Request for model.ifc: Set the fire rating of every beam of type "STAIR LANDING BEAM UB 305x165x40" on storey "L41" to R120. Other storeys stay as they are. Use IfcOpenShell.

First a look at what the model holds.

```python
import ifcopenshell
import ifcopenshell.util.element

model = ifcopenshell.open("model.ifc")
print(model.schema)
storey = next(s for s in model.by_type("IfcBuildingStorey") if s.Name == "L41")
beams = [e for e in ifcopenshell.util.element.get_decomposition(storey) if e.is_a("IfcBeam")]
seen = {}
for e in beams:
    element_type = ifcopenshell.util.element.get_type(e)
    key = (element_type.Name if element_type != e and element_type else None, ifcopenshell.util.element.get_pset(e, "Pset_BeamCommon", "FireRating"))
    seen[key] = seen.get(key, 0) + 1
for (name, value), count in sorted(seen.items(), key=str):
    print(count, "x", name, "|", value)
```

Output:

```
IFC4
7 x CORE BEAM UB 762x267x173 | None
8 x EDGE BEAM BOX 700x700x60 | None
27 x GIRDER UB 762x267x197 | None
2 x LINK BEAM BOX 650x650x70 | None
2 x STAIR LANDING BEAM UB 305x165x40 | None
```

```python
import ifcopenshell
import ifcopenshell.api.pset
import ifcopenshell.util.element

model = ifcopenshell.open("model.ifc")

storey = next(s for s in model.by_type("IfcBuildingStorey") if s.Name == "L41")
beams = [e for e in ifcopenshell.util.element.get_decomposition(storey) if e.is_a("IfcBeam")]

count = 0
for e in beams:
    element_type = ifcopenshell.util.element.get_type(e)
    if element_type in (None, e) or element_type.Name != "STAIR LANDING BEAM UB 305x165x40":
        continue
    found = ifcopenshell.util.element.get_pset(e, "Pset_BeamCommon", should_inherit=False)
    if found:
        pset = model.by_id(found["id"])
        if len(ifcopenshell.util.element.get_elements_by_pset(pset)) > 1:
            pset = ifcopenshell.api.pset.unshare_pset(model, products=[e], pset=pset)[0]
    else:
        pset = ifcopenshell.api.pset.add_pset(model, product=e, name="Pset_BeamCommon")
    ifcopenshell.api.pset.edit_pset(model, pset=pset, properties={"FireRating": "R120"})
    count += 1

print(count, "beams updated")

model.write("model_updated.ifc")
```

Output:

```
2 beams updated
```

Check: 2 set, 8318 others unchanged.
